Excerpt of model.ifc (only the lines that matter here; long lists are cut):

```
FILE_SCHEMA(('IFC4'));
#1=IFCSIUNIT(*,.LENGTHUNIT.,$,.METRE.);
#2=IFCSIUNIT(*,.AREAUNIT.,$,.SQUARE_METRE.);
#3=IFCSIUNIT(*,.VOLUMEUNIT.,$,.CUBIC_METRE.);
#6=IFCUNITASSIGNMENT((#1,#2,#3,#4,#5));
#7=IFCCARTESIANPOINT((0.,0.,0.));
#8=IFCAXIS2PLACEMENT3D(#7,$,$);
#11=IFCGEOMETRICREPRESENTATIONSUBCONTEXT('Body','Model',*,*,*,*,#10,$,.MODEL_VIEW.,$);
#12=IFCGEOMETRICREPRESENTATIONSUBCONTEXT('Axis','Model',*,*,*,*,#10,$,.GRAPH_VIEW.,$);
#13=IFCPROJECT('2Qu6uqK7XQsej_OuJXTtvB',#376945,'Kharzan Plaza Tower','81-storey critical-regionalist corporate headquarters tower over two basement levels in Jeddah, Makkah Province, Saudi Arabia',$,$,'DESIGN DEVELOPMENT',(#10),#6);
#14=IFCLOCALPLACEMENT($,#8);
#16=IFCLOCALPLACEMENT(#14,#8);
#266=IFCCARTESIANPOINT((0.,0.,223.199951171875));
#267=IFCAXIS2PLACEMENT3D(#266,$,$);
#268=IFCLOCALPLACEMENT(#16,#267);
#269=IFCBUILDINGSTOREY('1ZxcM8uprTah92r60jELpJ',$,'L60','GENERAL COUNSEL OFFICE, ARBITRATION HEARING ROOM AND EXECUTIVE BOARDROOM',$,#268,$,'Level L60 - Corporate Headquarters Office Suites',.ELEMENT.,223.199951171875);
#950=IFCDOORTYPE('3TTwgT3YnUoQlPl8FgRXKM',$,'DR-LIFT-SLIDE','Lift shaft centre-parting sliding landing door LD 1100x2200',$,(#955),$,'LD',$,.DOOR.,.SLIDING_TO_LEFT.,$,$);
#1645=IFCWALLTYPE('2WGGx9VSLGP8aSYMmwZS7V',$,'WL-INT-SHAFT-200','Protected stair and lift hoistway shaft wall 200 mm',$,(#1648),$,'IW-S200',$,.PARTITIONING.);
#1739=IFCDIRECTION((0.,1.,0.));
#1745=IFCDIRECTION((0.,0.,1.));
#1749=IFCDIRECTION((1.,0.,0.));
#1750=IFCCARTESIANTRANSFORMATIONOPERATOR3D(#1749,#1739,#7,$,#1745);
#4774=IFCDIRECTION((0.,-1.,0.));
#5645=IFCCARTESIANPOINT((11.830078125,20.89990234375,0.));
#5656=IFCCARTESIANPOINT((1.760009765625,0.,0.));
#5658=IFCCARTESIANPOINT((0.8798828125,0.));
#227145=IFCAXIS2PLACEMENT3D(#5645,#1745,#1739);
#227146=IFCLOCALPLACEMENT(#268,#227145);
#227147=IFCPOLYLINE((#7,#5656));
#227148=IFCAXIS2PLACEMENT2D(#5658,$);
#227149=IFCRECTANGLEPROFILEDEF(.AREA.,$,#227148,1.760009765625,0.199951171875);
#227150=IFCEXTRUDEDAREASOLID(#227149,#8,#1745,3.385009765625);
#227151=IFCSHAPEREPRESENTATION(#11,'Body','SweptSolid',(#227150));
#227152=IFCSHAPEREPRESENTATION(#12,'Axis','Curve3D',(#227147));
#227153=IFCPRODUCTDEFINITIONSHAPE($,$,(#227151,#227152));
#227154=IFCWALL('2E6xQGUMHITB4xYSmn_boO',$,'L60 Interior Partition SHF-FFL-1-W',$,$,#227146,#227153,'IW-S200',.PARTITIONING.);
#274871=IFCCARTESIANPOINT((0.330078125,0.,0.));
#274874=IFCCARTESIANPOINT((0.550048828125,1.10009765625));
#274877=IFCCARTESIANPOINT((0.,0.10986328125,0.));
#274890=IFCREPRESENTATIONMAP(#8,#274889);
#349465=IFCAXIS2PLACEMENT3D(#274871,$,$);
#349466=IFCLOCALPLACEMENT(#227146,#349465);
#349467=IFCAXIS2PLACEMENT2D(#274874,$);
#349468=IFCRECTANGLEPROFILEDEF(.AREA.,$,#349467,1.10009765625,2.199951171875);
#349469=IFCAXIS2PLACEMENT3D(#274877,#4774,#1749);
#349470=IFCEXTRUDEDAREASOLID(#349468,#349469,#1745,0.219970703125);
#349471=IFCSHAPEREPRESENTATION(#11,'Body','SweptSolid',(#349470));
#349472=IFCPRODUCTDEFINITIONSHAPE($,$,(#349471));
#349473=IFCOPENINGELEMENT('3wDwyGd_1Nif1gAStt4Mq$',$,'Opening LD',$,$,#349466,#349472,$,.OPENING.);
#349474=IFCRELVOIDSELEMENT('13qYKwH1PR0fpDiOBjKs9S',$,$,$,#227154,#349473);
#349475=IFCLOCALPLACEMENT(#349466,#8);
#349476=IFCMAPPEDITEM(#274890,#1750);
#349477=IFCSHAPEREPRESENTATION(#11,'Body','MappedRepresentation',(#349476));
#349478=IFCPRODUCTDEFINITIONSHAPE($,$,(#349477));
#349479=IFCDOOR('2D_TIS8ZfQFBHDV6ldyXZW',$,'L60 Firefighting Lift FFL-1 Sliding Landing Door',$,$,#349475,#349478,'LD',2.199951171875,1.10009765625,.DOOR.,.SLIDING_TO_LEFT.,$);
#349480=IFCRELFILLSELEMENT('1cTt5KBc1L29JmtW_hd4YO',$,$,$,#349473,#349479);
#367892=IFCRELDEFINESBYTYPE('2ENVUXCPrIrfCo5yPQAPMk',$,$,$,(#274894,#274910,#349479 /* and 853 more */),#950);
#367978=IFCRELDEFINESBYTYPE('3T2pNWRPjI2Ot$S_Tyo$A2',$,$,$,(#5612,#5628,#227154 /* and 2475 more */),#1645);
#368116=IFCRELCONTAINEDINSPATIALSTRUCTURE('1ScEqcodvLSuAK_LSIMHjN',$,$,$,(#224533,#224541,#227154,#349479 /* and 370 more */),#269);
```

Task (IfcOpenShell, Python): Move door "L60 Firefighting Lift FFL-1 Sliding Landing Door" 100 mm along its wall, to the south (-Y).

```python
import ifcopenshell
import ifcopenshell.api.geometry
import ifcopenshell.util.placement
import ifcopenshell.util.unit

model = ifcopenshell.open("model.ifc")
unit_scale = ifcopenshell.util.unit.calculate_unit_scale(model)

door = model.by_guid("2D_TIS8ZfQFBHDV6ldyXZW")
opening = door.FillsVoids[0].RelatingOpeningElement
wall = opening.VoidsElements[0].RelatingBuildingElement

wall_matrix = ifcopenshell.util.placement.get_local_placement(wall.ObjectPlacement)
shift = wall_matrix[:3, 0] * -0.1 / unit_scale
before = ifcopenshell.util.placement.get_local_placement(door.ObjectPlacement)[:3, 3].copy()

# The door is placed relative to its opening, so it follows when the opening moves.
matrix = ifcopenshell.util.placement.get_local_placement(opening.ObjectPlacement)
matrix[:3, 3] += shift
ifcopenshell.api.geometry.edit_object_placement(
    model, product=opening, matrix=matrix, is_si=False, should_transform_children=True
)

after = ifcopenshell.util.placement.get_local_placement(door.ObjectPlacement)[:3, 3]
print("door moved by", (after - before).round(3) + 0.0)

model.write("model_edited.ifc")
```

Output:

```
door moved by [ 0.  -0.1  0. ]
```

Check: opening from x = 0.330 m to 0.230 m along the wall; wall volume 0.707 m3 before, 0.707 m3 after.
